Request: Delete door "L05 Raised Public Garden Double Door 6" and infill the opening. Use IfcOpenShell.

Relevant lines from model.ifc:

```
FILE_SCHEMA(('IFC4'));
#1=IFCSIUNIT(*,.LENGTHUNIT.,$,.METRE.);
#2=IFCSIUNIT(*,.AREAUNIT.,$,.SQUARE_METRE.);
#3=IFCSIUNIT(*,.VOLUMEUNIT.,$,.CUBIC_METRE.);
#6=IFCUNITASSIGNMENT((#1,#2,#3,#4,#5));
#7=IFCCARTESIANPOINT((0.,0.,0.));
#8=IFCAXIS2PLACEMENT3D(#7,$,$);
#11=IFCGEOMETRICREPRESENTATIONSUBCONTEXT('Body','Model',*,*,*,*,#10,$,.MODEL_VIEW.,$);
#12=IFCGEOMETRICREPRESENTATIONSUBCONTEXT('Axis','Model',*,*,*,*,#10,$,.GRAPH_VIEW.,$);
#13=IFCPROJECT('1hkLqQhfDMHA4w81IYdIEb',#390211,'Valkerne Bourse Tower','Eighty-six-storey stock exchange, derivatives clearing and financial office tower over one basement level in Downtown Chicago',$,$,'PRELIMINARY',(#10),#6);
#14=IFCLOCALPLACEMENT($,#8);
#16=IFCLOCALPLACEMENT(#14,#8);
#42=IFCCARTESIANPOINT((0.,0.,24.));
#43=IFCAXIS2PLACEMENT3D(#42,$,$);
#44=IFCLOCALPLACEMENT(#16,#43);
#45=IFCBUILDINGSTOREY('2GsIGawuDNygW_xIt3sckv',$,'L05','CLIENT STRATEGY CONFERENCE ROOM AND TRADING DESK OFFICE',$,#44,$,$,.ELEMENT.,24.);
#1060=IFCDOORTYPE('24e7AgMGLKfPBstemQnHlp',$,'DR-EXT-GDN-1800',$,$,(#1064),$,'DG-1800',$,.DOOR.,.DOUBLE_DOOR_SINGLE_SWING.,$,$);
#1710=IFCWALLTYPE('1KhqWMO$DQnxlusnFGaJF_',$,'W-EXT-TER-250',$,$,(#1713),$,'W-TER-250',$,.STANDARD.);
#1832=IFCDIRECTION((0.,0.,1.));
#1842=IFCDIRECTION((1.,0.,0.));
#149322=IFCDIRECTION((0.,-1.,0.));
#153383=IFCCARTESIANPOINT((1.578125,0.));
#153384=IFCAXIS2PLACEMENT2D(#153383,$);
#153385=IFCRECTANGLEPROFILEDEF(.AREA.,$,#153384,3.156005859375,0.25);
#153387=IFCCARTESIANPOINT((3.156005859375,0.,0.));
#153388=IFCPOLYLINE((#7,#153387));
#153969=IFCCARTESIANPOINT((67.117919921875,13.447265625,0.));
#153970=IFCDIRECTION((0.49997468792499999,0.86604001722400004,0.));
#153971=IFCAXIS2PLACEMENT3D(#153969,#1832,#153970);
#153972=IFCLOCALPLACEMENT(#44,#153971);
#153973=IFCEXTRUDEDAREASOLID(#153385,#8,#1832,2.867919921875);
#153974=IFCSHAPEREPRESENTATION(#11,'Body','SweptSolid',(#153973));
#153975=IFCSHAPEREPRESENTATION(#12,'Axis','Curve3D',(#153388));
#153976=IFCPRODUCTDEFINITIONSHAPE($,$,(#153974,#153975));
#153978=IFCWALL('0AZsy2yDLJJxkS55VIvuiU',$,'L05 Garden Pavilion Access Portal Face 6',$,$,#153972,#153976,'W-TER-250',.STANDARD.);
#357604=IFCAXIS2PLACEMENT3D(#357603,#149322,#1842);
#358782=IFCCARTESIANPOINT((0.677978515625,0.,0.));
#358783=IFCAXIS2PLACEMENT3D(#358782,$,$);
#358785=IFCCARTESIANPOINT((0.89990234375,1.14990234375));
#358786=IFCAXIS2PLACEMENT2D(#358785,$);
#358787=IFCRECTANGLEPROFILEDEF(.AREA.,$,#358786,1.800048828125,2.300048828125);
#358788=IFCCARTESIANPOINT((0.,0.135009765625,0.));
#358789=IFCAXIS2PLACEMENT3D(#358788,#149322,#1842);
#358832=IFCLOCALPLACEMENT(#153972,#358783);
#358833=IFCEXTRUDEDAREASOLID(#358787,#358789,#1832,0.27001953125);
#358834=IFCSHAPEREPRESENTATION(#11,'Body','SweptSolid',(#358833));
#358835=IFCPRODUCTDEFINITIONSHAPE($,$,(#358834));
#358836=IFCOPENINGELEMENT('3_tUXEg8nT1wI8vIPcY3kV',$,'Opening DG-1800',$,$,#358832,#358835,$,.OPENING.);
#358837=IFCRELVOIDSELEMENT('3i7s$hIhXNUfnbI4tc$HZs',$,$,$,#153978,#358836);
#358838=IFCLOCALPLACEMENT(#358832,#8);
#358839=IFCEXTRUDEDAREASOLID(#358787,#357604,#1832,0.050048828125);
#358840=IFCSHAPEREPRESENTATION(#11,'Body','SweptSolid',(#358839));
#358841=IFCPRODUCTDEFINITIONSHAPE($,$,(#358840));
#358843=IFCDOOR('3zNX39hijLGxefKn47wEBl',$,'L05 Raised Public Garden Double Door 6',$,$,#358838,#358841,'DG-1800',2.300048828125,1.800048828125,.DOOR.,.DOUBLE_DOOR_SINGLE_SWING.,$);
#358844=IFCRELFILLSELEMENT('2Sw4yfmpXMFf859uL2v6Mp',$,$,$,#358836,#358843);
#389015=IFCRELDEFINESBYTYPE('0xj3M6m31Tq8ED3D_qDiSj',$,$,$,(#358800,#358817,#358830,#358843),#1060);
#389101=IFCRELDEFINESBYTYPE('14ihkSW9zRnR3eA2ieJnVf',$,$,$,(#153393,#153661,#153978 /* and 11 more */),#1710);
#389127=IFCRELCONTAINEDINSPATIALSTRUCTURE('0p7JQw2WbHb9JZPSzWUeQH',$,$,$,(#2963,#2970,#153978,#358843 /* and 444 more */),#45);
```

```python
import ifcopenshell
import ifcopenshell.api.feature
import ifcopenshell.api.root
import ifcopenshell.geom
import ifcopenshell.util.shape

model = ifcopenshell.open("model.ifc")
settings = ifcopenshell.geom.settings()


def volume(element):
    """Net volume in cubic metres, openings subtracted."""
    shape = ifcopenshell.geom.create_shape(settings, element)
    return ifcopenshell.util.shape.get_volume(shape.geometry)


door = model.by_guid("3zNX39hijLGxefKn47wEBl")
opening = door.FillsVoids[0].RelatingOpeningElement
wall = opening.VoidsElements[0].RelatingBuildingElement
before = volume(wall)

ifcopenshell.api.root.remove_product(model, product=door)
ifcopenshell.api.feature.remove_feature(model, feature=opening)

after = volume(wall)

print(f"wall volume {before:.3f} -> {after:.3f} m3")

model.write("model_edited.ifc")
```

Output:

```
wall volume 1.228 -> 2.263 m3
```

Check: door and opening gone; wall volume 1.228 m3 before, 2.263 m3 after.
